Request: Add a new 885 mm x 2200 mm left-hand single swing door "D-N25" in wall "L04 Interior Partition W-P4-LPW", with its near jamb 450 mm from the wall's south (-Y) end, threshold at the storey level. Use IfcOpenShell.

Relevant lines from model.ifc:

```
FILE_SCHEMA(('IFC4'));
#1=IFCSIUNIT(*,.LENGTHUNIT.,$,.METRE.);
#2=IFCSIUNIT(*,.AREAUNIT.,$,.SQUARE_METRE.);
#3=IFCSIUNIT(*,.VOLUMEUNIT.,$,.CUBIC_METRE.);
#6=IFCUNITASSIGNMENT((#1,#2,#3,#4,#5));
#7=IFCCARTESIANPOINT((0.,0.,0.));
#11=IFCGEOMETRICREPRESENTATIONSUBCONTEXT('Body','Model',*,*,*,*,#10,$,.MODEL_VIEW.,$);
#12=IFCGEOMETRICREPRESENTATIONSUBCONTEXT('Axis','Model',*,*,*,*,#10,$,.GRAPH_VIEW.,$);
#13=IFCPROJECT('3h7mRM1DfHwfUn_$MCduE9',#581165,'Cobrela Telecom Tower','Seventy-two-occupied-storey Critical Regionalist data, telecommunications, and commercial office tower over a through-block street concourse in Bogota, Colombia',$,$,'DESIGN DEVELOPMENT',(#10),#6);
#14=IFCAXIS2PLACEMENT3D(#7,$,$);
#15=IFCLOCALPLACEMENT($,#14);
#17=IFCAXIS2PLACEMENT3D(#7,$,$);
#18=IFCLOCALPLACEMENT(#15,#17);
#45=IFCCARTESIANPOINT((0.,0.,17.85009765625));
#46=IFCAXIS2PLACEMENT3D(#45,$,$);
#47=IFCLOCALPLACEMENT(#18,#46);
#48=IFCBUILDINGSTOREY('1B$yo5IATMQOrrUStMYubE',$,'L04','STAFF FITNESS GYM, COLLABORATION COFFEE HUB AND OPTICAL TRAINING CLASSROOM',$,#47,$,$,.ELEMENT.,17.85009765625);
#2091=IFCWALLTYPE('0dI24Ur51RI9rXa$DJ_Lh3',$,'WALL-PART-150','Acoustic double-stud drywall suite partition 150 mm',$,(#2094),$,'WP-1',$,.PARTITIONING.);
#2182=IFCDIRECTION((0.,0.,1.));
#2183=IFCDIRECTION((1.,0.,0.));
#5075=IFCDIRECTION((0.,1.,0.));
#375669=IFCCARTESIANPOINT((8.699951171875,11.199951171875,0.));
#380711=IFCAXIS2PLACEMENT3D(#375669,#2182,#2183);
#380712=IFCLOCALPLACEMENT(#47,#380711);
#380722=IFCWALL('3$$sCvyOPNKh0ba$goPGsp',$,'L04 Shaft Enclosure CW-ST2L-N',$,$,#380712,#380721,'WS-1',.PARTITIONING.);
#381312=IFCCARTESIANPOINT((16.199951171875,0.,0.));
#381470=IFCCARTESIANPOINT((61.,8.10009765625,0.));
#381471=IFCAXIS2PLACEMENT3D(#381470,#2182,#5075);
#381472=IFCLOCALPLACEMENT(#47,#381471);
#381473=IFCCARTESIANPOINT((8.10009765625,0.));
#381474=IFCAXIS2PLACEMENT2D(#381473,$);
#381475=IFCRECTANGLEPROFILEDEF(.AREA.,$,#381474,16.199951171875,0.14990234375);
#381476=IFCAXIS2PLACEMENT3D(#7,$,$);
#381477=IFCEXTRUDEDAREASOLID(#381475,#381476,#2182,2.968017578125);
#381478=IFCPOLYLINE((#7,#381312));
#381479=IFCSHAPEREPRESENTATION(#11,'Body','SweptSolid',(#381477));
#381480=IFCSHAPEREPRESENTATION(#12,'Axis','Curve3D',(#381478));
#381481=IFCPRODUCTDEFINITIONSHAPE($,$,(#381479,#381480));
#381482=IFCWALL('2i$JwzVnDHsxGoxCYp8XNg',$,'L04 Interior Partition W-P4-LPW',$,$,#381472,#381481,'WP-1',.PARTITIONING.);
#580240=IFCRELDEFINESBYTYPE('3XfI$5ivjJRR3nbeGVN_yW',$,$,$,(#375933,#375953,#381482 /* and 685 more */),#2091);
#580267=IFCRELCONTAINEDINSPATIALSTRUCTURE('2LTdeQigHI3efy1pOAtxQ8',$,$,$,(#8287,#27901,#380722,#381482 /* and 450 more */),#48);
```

```python
import numpy as np
import ifcopenshell
import ifcopenshell.api.feature
import ifcopenshell.api.geometry
import ifcopenshell.api.root
import ifcopenshell.api.spatial
import ifcopenshell.geom
import ifcopenshell.util.element
import ifcopenshell.util.placement
import ifcopenshell.util.representation
import ifcopenshell.util.shape
import ifcopenshell.util.unit

model = ifcopenshell.open("model.ifc")
unit_scale = ifcopenshell.util.unit.calculate_unit_scale(model)
settings = ifcopenshell.geom.settings()


def volume(element):
    """Net volume in cubic metres, openings subtracted."""
    shape = ifcopenshell.geom.create_shape(settings, element)
    return ifcopenshell.util.shape.get_volume(shape.geometry)


wall = model.by_guid("2i$JwzVnDHsxGoxCYp8XNg")
storey = ifcopenshell.util.element.get_container(wall, ifc_class="IfcBuildingStorey")
context = ifcopenshell.util.representation.get_context(model, "Model", "Body", "MODEL_VIEW")
before = volume(wall)

width, height, from_end, sill = 0.885, 2.2, 0.45, 0.0  # metres

# The wall runs along its own X axis, and the end named is its -X end.
wall_shape = ifcopenshell.geom.create_shape(settings, wall)
x, y, z = ifcopenshell.util.shape.get_vertices(wall_shape.geometry).T
start = x.min() + from_end
face, thickness = float(y.min()), float(y.max() - y.min())
wall_matrix = ifcopenshell.util.placement.get_local_placement(wall.ObjectPlacement)
level = ifcopenshell.util.placement.get_local_placement(storey.ObjectPlacement)[2, 3]


def in_wall(x, y):
    """Placement at x, y metres in the wall's axes, at sill height."""
    matrix = wall_matrix.copy()
    matrix[:, 3] = wall_matrix @ np.array([x / unit_scale, y / unit_scale, 0.0, 1.0])
    matrix[2, 3] = level + sill / unit_scale
    return matrix


# Opening: a box that overshoots both wall faces by 50 mm.
opening = ifcopenshell.api.root.create_entity(model, ifc_class="IfcOpeningElement", predefined_type="OPENING")
box = ifcopenshell.api.geometry.add_wall_representation(
    model, context=context, length=width, height=height, thickness=thickness + 0.1
)
ifcopenshell.api.geometry.assign_representation(model, product=opening, representation=box)
ifcopenshell.api.geometry.edit_object_placement(model, product=opening, matrix=in_wall(start, face - 0.05), is_si=False)
ifcopenshell.api.feature.add_feature(model, feature=opening, element=wall)

door = ifcopenshell.api.root.create_entity(model, ifc_class="IfcDoor", name="D-N25", predefined_type="DOOR")
door.OverallWidth, door.OverallHeight = width / unit_scale, height / unit_scale
door.OperationType = "SINGLE_SWING_LEFT"
body = ifcopenshell.api.geometry.add_door_representation(
    model,
    context=context,
    overall_width=door.OverallWidth,
    overall_height=door.OverallHeight,
    operation_type="SINGLE_SWING_LEFT",
    lining_properties={"LiningDepth": thickness / unit_scale, "ThresholdDepth": thickness / unit_scale},
)
ifcopenshell.api.geometry.assign_representation(model, product=door, representation=body)
ifcopenshell.api.spatial.assign_container(model, products=[door], relating_structure=storey)
ifcopenshell.api.feature.add_filling(model, opening=opening, element=door)

# The lining spans the wall, so the door starts at the wall face.
ifcopenshell.api.geometry.edit_object_placement(model, product=door, matrix=in_wall(start, face), is_si=False)

after = volume(wall)

print(f"wall volume {before:.3f} -> {after:.3f} m3")

model.write("model_v2.ifc")
```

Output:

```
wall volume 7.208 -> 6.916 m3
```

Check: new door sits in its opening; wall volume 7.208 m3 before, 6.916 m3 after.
